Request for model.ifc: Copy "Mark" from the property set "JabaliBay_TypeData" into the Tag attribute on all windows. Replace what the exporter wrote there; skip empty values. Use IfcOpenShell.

First a look at what the model holds.

```python
import ifcopenshell
import ifcopenshell.util.element

model = ifcopenshell.open("model.ifc")
print(model.schema)
windows = model.by_type("IfcWindow")
print(len(windows), "windows")
for e in windows[:8]:
    source = ifcopenshell.util.element.get_pset(e, "JabaliBay_TypeData", "Mark")
    target = e.Tag
    print(e.id(), repr(source), repr(target), sep=" | ")
```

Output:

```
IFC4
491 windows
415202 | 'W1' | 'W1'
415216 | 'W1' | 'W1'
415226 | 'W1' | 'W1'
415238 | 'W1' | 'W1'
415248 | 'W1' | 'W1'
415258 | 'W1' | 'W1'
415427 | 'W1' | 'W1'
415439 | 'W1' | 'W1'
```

```python
import ifcopenshell
import ifcopenshell.util.element

model = ifcopenshell.open("model.ifc")

count = 0
for e in model.by_type("IfcWindow"):
    value = ifcopenshell.util.element.get_pset(e, "JabaliBay_TypeData", "Mark")
    current = e.Tag
    if not value or not value.strip() or current == value:
        continue
    e.Tag = value
    count += 1

print(count, "windows updated")

model.write("model_updated.ifc")
```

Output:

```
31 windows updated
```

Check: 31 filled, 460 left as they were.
